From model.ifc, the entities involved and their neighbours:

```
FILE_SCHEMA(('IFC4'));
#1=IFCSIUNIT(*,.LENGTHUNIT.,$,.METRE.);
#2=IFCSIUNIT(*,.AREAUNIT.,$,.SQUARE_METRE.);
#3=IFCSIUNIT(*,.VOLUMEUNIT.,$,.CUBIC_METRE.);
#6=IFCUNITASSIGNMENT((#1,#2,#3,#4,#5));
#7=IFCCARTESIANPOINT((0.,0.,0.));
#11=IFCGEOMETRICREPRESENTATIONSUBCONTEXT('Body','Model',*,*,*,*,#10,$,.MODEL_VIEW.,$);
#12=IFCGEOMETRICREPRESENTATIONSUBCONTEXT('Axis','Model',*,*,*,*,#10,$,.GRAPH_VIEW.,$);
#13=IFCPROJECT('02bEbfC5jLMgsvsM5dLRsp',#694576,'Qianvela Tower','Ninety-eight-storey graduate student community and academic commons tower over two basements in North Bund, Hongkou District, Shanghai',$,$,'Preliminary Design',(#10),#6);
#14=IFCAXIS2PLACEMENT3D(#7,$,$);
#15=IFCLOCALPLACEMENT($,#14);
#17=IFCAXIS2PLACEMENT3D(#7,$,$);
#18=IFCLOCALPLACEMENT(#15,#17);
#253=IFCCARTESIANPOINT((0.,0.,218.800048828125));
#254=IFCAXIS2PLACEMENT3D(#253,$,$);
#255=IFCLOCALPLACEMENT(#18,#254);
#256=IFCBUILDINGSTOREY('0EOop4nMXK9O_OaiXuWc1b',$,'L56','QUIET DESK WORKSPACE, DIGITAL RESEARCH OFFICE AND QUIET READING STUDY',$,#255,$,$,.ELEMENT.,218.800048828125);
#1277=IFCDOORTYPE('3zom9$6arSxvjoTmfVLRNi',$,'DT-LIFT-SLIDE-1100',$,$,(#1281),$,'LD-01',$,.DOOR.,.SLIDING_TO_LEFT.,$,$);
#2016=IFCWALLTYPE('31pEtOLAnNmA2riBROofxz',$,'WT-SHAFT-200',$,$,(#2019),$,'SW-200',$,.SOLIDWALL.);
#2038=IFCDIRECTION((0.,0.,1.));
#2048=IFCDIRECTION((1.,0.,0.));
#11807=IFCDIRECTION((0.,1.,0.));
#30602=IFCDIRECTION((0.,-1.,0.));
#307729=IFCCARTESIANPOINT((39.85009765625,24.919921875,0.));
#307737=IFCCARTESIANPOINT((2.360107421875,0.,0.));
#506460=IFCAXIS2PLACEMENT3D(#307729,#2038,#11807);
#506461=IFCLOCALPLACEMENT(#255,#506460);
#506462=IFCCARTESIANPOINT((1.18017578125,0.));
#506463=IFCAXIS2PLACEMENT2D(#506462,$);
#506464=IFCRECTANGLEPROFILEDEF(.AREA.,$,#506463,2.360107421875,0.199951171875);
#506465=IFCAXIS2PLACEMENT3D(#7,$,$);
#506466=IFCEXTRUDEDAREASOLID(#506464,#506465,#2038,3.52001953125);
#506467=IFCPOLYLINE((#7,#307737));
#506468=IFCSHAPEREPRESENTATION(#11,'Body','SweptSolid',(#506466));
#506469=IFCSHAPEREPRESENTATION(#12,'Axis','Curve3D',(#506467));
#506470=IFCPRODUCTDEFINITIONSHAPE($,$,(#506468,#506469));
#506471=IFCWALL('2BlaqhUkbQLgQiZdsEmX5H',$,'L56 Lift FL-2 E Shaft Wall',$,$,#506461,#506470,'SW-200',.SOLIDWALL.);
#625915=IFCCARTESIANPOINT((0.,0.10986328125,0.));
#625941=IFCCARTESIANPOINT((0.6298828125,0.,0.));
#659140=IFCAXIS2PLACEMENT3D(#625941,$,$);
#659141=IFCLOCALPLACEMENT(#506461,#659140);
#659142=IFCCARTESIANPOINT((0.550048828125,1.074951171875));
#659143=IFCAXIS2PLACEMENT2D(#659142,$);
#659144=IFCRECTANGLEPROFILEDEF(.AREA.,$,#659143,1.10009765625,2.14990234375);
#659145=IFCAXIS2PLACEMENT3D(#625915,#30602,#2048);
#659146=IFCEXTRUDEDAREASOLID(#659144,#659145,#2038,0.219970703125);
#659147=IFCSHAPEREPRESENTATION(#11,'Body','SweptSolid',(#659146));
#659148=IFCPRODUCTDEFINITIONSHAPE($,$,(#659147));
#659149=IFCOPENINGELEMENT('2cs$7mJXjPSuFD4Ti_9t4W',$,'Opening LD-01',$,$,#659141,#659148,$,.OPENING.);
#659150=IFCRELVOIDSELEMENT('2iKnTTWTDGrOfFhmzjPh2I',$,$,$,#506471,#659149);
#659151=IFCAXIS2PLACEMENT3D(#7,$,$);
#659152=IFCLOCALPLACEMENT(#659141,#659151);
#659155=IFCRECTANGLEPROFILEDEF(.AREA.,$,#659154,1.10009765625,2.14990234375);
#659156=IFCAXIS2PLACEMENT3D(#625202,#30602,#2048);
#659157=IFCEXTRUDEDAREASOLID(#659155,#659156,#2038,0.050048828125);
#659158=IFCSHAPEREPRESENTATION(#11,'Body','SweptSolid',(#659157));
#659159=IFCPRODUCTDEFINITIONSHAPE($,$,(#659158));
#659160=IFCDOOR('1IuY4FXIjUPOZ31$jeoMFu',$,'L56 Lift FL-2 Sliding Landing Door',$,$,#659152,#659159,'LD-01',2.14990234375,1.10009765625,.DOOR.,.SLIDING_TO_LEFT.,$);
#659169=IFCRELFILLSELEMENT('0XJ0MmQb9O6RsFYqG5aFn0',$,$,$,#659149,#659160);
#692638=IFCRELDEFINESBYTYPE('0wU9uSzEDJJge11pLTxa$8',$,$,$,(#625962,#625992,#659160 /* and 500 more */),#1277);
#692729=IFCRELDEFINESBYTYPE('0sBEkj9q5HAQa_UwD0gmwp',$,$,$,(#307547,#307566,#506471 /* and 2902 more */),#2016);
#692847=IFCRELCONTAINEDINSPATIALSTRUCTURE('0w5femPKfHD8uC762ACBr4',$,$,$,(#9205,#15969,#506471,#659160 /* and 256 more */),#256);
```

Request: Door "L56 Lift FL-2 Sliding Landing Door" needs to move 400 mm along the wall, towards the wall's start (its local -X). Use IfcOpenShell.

```python
import ifcopenshell
import ifcopenshell.api.geometry
import ifcopenshell.util.placement

model = ifcopenshell.open("model.ifc")

door = model.by_id(659160)
opening = door.FillsVoids[0].RelatingOpeningElement
wall = opening.VoidsElements[0].RelatingBuildingElement

wall_matrix = ifcopenshell.util.placement.get_local_placement(wall.ObjectPlacement)
shift = wall_matrix[:3, 0] * -0.4
before = ifcopenshell.util.placement.get_local_placement(door.ObjectPlacement)[:3, 3].copy()

# The door is placed relative to its opening, so it follows when the opening moves.
matrix = ifcopenshell.util.placement.get_local_placement(opening.ObjectPlacement)
matrix[:3, 3] += shift
ifcopenshell.api.geometry.edit_object_placement(
    model, product=opening, matrix=matrix, is_si=False, should_transform_children=True
)

after = ifcopenshell.util.placement.get_local_placement(door.ObjectPlacement)[:3, 3]
print("door moved by", (after - before).round(3) + 0.0)

model.write("model_v2.ifc")
```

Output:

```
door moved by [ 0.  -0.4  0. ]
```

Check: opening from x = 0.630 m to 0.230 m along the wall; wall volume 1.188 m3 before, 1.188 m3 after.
